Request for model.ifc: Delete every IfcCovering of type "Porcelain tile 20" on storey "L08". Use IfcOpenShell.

First a look at what the model holds.

```python
import ifcopenshell
import ifcopenshell.util.element

model = ifcopenshell.open("model.ifc")
print(model.schema)
storey = next(s for s in model.by_type("IfcBuildingStorey") if s.Name == "L08")
coverings = [e for e in ifcopenshell.util.element.get_decomposition(storey) if e.is_a("IfcCovering")]
seen = {}
for e in coverings:
    element_type = ifcopenshell.util.element.get_type(e)
    name = element_type.Name if element_type not in (None, e) else None
    seen[name] = seen.get(name, 0) + 1
for name, count in sorted(seen.items(), key=str):
    print(count, "x", name)
```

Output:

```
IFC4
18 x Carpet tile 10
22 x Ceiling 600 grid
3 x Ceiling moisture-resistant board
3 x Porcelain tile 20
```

```python
import ifcopenshell
import ifcopenshell.api.root
import ifcopenshell.util.element

model = ifcopenshell.open("model.ifc")

storey = next(s for s in model.by_type("IfcBuildingStorey") if s.Name == "L08")
coverings = [e for e in ifcopenshell.util.element.get_decomposition(storey) if e.is_a("IfcCovering")]
targets = [e for e in coverings if (t := ifcopenshell.util.element.get_type(e)) not in (None, e) and t.Name == "Porcelain tile 20"]

for e in targets:
    ifcopenshell.api.root.remove_product(model, product=e)
print(len(targets), "removed")

model.write("model_updated.ifc")
```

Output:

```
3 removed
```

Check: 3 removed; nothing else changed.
